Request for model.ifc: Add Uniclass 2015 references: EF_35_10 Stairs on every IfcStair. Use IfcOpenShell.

First a look at what the model holds.

```python
import ifcopenshell

model = ifcopenshell.open("model.ifc")
print(model.schema)
print("classifications:", [c.Name for c in model.by_type("IfcClassification")])
for ifc_class in ("IfcDoor", "IfcRoof", "IfcStair", "IfcWall", "IfcWindow"):
    print(ifc_class, len(model.by_type(ifc_class)))
```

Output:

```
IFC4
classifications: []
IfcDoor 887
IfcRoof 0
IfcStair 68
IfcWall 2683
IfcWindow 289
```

```python
import ifcopenshell
import ifcopenshell.api.classification

model = ifcopenshell.open("model.ifc")

system = ifcopenshell.api.classification.add_classification(model, classification="Uniclass 2015")

codes = {
    "IfcStair": ("EF_35_10", "Stairs"),
}
for ifc_class, (code, name) in codes.items():
    products = model.by_type(ifc_class)
    ifcopenshell.api.classification.add_reference(
        model, products=products, classification=system, identification=code, name=name
    )
    print(code, len(products))

model.write("model_v2.ifc")
```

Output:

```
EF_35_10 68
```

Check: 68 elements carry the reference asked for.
